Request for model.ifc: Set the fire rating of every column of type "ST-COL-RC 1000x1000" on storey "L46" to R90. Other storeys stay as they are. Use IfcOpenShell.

First a look at what the model holds.

```python
import ifcopenshell
import ifcopenshell.util.element

model = ifcopenshell.open("model.ifc")
print(model.schema)
storey = next(s for s in model.by_type("IfcBuildingStorey") if s.Name == "L46")
columns = [e for e in ifcopenshell.util.element.get_decomposition(storey) if e.is_a("IfcColumn")]
seen = {}
for e in columns:
    element_type = ifcopenshell.util.element.get_type(e)
    key = (element_type.Name if element_type != e and element_type else None, ifcopenshell.util.element.get_pset(e, "Pset_ColumnCommon", "FireRating"))
    seen[key] = seen.get(key, 0) + 1
for (name, value), count in sorted(seen.items(), key=str):
    print(count, "x", name, "|", value)
```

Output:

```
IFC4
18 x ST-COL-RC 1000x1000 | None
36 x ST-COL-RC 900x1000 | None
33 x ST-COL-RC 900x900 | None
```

```python
import ifcopenshell
import ifcopenshell.api.pset
import ifcopenshell.util.element

model = ifcopenshell.open("model.ifc")

storey = next(s for s in model.by_type("IfcBuildingStorey") if s.Name == "L46")
columns = [e for e in ifcopenshell.util.element.get_decomposition(storey) if e.is_a("IfcColumn")]

count = 0
for e in columns:
    element_type = ifcopenshell.util.element.get_type(e)
    if element_type in (None, e) or element_type.Name != "ST-COL-RC 1000x1000":
        continue
    found = ifcopenshell.util.element.get_pset(e, "Pset_ColumnCommon", should_inherit=False)
    if found:
        pset = model.by_id(found["id"])
        if len(ifcopenshell.util.element.get_elements_by_pset(pset)) > 1:
            pset = ifcopenshell.api.pset.unshare_pset(model, products=[e], pset=pset)[0]
    else:
        pset = ifcopenshell.api.pset.add_pset(model, product=e, name="Pset_ColumnCommon")
    ifcopenshell.api.pset.edit_pset(model, pset=pset, properties={"FireRating": "R90"})
    count += 1

print(count, "columns updated")

model.write("model_rev.ifc")
```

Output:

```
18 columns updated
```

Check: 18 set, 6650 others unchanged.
